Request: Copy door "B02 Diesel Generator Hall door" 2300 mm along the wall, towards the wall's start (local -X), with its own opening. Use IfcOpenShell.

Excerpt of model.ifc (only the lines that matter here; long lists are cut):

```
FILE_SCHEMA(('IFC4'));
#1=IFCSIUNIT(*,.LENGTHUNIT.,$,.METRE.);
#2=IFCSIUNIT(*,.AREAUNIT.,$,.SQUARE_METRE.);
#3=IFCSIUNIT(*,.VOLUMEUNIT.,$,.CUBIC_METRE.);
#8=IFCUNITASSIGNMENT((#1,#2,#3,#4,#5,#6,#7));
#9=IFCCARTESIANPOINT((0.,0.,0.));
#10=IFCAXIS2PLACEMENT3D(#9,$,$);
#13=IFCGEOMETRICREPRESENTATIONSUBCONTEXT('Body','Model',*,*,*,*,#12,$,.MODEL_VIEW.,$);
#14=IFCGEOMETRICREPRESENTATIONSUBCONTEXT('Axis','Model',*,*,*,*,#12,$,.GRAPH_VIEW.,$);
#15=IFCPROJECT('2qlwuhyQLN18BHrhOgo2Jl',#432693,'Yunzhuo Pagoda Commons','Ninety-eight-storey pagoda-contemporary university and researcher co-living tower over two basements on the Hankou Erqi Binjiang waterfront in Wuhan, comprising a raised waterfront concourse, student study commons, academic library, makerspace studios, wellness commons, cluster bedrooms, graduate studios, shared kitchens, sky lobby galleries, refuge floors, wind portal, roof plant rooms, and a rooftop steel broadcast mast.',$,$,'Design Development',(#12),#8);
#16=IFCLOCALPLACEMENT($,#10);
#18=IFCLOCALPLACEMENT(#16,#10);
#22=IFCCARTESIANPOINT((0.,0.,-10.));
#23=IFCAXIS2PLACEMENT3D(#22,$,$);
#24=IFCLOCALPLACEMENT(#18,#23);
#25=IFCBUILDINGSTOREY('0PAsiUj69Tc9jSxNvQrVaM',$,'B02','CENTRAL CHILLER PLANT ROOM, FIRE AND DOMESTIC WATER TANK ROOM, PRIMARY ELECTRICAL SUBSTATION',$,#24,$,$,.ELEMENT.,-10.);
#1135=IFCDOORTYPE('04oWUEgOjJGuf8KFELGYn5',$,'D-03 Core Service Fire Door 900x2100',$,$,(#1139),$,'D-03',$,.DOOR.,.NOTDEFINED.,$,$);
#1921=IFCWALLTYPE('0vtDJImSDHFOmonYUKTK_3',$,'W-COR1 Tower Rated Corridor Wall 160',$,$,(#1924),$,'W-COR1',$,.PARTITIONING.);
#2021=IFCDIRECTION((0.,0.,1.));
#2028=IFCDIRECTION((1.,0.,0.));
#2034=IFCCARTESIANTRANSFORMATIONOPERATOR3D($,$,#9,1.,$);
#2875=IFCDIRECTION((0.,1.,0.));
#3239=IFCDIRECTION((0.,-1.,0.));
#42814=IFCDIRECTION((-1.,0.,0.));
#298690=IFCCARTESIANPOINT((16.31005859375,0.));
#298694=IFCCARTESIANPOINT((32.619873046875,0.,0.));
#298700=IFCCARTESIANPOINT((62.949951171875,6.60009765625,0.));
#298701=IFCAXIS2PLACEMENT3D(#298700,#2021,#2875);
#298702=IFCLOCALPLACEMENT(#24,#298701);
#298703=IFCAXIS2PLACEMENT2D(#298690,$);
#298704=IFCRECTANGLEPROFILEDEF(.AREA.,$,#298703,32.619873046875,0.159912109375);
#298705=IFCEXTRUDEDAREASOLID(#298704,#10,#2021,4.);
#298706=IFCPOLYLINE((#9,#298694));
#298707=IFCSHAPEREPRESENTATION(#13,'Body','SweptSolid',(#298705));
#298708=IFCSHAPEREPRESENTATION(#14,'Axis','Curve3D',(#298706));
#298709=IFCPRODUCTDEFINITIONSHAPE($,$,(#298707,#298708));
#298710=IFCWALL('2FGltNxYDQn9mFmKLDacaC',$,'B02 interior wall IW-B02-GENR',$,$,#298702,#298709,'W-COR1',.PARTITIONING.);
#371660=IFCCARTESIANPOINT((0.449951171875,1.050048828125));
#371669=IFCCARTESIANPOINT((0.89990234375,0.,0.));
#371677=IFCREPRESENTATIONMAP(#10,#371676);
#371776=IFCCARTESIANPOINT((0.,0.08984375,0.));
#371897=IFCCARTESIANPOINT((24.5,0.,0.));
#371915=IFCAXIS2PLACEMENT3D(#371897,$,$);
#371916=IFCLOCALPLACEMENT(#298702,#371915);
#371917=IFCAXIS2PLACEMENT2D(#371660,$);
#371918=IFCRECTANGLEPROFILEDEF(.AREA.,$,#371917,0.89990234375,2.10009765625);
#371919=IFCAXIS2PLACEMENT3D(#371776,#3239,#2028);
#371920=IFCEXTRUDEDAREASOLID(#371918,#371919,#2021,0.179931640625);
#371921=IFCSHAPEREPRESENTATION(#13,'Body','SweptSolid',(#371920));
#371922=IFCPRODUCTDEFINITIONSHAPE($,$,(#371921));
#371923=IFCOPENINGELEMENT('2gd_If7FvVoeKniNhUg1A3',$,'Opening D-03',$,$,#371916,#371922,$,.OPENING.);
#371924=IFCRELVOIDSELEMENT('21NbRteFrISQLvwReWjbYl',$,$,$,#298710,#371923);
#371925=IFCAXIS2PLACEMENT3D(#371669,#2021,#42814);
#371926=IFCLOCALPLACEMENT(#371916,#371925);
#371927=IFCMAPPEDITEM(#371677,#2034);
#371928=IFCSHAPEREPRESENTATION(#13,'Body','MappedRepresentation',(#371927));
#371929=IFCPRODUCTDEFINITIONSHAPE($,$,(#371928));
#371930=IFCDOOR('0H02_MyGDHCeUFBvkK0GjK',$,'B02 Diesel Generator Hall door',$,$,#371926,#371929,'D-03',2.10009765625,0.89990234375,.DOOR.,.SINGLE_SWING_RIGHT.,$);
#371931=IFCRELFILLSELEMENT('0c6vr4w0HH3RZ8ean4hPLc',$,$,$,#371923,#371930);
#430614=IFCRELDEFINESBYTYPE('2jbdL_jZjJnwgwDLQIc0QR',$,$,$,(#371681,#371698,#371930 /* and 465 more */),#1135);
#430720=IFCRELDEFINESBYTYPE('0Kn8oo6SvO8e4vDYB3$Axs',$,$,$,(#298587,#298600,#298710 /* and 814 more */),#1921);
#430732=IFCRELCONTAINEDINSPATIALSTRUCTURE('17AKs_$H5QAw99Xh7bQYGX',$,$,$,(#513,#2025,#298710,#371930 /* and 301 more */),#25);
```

```python
import ifcopenshell
import ifcopenshell.api.feature
import ifcopenshell.api.geometry
import ifcopenshell.api.root
import ifcopenshell.geom
import ifcopenshell.util.element
import ifcopenshell.util.placement
import ifcopenshell.util.shape

model = ifcopenshell.open("model.ifc")
settings = ifcopenshell.geom.settings()


def volume(element):
    """Net volume in cubic metres, openings subtracted."""
    shape = ifcopenshell.geom.create_shape(settings, element)
    return ifcopenshell.util.shape.get_volume(shape.geometry)


door = model.by_guid("0H02_MyGDHCeUFBvkK0GjK")
opening = door.FillsVoids[0].RelatingOpeningElement
wall = opening.VoidsElements[0].RelatingBuildingElement
before = volume(wall)
shift = ifcopenshell.util.placement.get_local_placement(wall.ObjectPlacement)[:3, 0] * -2.3

# copy_class copies the void relationship, type, container and properties, but no geometry.
new_opening = ifcopenshell.api.root.copy_class(model, product=opening)
new_opening.Representation = ifcopenshell.util.element.copy_deep(
    model, opening.Representation, exclude=["IfcGeometricRepresentationContext", "IfcRepresentationMap"]
)
new_door = ifcopenshell.api.root.copy_class(model, product=door)
new_door.Representation = ifcopenshell.util.element.copy_deep(
    model, door.Representation, exclude=["IfcGeometricRepresentationContext", "IfcRepresentationMap"]
)
new_door.Tag = None
ifcopenshell.api.feature.add_filling(model, opening=new_opening, element=new_door)

for old, new in ((opening, new_opening), (door, new_door)):
    matrix = ifcopenshell.util.placement.get_local_placement(old.ObjectPlacement)
    matrix[:3, 3] += shift
    ifcopenshell.api.geometry.edit_object_placement(model, product=new, matrix=matrix, is_si=False)

after = volume(wall)

print(f"wall volume {before:.3f} -> {after:.3f} m3")

model.write("model_updated.ifc")
```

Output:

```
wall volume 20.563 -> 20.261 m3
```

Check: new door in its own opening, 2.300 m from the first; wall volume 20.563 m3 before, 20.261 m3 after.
